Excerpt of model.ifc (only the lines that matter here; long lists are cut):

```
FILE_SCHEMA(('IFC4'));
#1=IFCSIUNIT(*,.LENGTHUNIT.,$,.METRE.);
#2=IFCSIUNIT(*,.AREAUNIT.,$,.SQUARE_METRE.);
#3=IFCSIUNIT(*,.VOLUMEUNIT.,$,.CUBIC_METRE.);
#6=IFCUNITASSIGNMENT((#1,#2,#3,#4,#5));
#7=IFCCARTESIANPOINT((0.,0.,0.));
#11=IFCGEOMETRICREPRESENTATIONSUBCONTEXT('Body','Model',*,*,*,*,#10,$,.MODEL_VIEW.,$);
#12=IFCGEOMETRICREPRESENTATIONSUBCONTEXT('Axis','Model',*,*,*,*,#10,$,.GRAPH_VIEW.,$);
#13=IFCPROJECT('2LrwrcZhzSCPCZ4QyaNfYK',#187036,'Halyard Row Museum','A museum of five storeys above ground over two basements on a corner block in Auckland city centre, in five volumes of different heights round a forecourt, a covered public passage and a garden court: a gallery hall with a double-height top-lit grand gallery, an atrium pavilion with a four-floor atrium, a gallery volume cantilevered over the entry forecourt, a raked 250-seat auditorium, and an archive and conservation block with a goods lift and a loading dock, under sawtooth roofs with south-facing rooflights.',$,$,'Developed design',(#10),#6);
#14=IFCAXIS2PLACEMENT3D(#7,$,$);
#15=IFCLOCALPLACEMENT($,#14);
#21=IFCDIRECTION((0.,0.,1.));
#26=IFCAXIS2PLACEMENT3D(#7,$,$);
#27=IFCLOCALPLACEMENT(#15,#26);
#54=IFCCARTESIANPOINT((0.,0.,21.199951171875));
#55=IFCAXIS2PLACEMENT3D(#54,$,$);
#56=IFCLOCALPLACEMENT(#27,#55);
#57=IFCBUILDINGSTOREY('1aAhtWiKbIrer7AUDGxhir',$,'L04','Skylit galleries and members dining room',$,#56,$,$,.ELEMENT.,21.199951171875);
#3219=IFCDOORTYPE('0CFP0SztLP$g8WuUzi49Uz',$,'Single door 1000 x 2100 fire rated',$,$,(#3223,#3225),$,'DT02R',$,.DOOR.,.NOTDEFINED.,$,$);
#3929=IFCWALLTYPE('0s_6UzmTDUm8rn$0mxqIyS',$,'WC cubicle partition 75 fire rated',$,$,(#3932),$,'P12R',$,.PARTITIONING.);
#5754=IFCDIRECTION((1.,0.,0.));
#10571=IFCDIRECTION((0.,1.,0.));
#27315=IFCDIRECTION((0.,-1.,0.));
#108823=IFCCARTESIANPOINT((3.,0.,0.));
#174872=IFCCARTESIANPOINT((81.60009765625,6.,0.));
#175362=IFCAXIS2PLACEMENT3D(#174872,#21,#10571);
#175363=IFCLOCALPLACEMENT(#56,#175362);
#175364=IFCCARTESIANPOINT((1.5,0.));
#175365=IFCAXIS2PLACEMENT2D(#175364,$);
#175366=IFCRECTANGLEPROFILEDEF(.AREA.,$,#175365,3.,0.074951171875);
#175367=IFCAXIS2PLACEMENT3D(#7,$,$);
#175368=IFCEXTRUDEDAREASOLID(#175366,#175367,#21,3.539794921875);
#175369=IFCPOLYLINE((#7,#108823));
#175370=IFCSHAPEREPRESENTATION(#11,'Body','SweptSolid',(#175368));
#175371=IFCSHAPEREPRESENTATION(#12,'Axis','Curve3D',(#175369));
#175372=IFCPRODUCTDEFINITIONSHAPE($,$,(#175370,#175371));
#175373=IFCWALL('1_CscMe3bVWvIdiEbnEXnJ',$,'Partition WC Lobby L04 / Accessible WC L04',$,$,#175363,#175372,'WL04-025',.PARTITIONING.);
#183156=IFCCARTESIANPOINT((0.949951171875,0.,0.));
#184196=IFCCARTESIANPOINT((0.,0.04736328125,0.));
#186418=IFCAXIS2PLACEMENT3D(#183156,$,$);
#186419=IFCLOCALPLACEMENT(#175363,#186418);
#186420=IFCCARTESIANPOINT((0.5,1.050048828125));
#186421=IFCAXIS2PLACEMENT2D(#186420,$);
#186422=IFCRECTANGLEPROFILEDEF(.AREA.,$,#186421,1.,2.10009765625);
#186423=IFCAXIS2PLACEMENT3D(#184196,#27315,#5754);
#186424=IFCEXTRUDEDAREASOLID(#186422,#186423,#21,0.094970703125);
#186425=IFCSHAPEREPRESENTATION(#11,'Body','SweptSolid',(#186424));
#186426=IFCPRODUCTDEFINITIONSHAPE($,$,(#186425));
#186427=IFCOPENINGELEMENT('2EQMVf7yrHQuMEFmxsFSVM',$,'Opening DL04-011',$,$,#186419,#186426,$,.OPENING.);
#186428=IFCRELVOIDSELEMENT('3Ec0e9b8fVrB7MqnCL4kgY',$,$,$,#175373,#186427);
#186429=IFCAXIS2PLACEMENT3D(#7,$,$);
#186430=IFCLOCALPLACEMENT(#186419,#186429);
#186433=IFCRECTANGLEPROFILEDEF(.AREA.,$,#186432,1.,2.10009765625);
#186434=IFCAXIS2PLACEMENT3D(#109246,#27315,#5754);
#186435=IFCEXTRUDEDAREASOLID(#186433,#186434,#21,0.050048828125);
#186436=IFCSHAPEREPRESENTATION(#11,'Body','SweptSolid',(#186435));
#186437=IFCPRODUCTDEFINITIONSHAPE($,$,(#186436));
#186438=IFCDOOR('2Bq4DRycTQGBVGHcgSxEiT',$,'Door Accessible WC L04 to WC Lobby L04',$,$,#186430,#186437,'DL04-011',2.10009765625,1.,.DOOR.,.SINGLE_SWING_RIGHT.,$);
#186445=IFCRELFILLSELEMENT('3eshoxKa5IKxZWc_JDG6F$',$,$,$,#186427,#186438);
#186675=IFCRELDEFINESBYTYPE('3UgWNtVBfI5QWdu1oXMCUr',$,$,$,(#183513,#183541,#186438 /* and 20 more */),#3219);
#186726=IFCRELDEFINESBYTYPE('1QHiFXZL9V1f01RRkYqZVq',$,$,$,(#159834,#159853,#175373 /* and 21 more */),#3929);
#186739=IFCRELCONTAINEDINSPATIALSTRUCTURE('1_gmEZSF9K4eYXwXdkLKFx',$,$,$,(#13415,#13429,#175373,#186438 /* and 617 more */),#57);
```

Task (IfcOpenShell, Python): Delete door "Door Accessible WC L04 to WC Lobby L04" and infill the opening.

```python
import ifcopenshell
import ifcopenshell.api.feature
import ifcopenshell.api.root
import ifcopenshell.geom
import ifcopenshell.util.shape

model = ifcopenshell.open("model.ifc")
settings = ifcopenshell.geom.settings()


def volume(element):
    """Net volume in cubic metres, openings subtracted."""
    shape = ifcopenshell.geom.create_shape(settings, element)
    return ifcopenshell.util.shape.get_volume(shape.geometry)


door = model.by_guid("2Bq4DRycTQGBVGHcgSxEiT")
opening = door.FillsVoids[0].RelatingOpeningElement
wall = opening.VoidsElements[0].RelatingBuildingElement
before = volume(wall)

ifcopenshell.api.root.remove_product(model, product=door)
ifcopenshell.api.feature.remove_feature(model, feature=opening)

after = volume(wall)

print(f"wall volume {before:.3f} -> {after:.3f} m3")

model.write("model_edited.ifc")
```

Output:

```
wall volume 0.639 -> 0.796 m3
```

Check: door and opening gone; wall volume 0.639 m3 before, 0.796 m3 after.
